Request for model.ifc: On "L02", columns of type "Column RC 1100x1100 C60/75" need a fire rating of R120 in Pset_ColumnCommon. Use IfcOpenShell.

First a look at what the model holds.

```python
import ifcopenshell
import ifcopenshell.util.element

model = ifcopenshell.open("model.ifc")
print(model.schema)
storey = next(s for s in model.by_type("IfcBuildingStorey") if s.Name == "L02")
columns = [e for e in ifcopenshell.util.element.get_decomposition(storey) if e.is_a("IfcColumn")]
seen = {}
for e in columns:
    element_type = ifcopenshell.util.element.get_type(e)
    key = (element_type.Name if element_type != e and element_type else None, ifcopenshell.util.element.get_pset(e, "Pset_ColumnCommon", "FireRating"))
    seen[key] = seen.get(key, 0) + 1
for (name, value), count in sorted(seen.items(), key=str):
    print(count, "x", name, "|", value)
```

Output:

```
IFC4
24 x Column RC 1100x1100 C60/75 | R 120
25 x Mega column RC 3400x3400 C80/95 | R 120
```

```python
import ifcopenshell
import ifcopenshell.api.pset
import ifcopenshell.util.element

model = ifcopenshell.open("model.ifc")

storey = next(s for s in model.by_type("IfcBuildingStorey") if s.Name == "L02")
columns = [e for e in ifcopenshell.util.element.get_decomposition(storey) if e.is_a("IfcColumn")]

count = 0
for e in columns:
    element_type = ifcopenshell.util.element.get_type(e)
    if element_type in (None, e) or element_type.Name != "Column RC 1100x1100 C60/75":
        continue
    # add_pset returns the element's existing set when there is one.
    pset = ifcopenshell.api.pset.add_pset(model, product=e, name="Pset_ColumnCommon")
    ifcopenshell.api.pset.edit_pset(model, pset=pset, properties={"FireRating": "R120"})
    count += 1

print(count, "columns updated")

model.write("model_edited.ifc")
```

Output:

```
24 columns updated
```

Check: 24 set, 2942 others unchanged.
